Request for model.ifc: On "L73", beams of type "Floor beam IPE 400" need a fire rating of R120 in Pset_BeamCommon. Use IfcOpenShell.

First a look at what the model holds.

```python
import ifcopenshell
import ifcopenshell.util.element

model = ifcopenshell.open("model.ifc")
print(model.schema)
storey = next(s for s in model.by_type("IfcBuildingStorey") if s.Name == "L73")
beams = [e for e in ifcopenshell.util.element.get_decomposition(storey) if e.is_a("IfcBeam")]
seen = {}
for e in beams:
    element_type = ifcopenshell.util.element.get_type(e)
    key = (element_type.Name if element_type != e and element_type else None, ifcopenshell.util.element.get_pset(e, "Pset_BeamCommon", "FireRating"))
    seen[key] = seen.get(key, 0) + 1
for (name, value), count in sorted(seen.items(), key=str):
    print(count, "x", name, "|", value)
```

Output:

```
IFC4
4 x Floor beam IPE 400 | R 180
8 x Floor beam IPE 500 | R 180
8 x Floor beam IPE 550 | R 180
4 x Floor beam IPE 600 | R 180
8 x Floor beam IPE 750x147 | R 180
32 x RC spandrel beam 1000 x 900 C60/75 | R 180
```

```python
import ifcopenshell
import ifcopenshell.api.pset
import ifcopenshell.util.element

model = ifcopenshell.open("model.ifc")

storey = next(s for s in model.by_type("IfcBuildingStorey") if s.Name == "L73")
beams = [e for e in ifcopenshell.util.element.get_decomposition(storey) if e.is_a("IfcBeam")]

count = 0
for e in beams:
    element_type = ifcopenshell.util.element.get_type(e)
    if element_type in (None, e) or element_type.Name != "Floor beam IPE 400":
        continue
    found = ifcopenshell.util.element.get_pset(e, "Pset_BeamCommon", should_inherit=False)
    if found:
        pset = model.by_id(found["id"])
        if len(ifcopenshell.util.element.get_elements_by_pset(pset)) > 1:
            pset = ifcopenshell.api.pset.unshare_pset(model, products=[e], pset=pset)[0]
    else:
        pset = ifcopenshell.api.pset.add_pset(model, product=e, name="Pset_BeamCommon")
    ifcopenshell.api.pset.edit_pset(model, pset=pset, properties={"FireRating": "R120"})
    count += 1

print(count, "beams updated")

model.write("model_edited.ifc")
```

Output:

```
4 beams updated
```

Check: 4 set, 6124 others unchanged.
